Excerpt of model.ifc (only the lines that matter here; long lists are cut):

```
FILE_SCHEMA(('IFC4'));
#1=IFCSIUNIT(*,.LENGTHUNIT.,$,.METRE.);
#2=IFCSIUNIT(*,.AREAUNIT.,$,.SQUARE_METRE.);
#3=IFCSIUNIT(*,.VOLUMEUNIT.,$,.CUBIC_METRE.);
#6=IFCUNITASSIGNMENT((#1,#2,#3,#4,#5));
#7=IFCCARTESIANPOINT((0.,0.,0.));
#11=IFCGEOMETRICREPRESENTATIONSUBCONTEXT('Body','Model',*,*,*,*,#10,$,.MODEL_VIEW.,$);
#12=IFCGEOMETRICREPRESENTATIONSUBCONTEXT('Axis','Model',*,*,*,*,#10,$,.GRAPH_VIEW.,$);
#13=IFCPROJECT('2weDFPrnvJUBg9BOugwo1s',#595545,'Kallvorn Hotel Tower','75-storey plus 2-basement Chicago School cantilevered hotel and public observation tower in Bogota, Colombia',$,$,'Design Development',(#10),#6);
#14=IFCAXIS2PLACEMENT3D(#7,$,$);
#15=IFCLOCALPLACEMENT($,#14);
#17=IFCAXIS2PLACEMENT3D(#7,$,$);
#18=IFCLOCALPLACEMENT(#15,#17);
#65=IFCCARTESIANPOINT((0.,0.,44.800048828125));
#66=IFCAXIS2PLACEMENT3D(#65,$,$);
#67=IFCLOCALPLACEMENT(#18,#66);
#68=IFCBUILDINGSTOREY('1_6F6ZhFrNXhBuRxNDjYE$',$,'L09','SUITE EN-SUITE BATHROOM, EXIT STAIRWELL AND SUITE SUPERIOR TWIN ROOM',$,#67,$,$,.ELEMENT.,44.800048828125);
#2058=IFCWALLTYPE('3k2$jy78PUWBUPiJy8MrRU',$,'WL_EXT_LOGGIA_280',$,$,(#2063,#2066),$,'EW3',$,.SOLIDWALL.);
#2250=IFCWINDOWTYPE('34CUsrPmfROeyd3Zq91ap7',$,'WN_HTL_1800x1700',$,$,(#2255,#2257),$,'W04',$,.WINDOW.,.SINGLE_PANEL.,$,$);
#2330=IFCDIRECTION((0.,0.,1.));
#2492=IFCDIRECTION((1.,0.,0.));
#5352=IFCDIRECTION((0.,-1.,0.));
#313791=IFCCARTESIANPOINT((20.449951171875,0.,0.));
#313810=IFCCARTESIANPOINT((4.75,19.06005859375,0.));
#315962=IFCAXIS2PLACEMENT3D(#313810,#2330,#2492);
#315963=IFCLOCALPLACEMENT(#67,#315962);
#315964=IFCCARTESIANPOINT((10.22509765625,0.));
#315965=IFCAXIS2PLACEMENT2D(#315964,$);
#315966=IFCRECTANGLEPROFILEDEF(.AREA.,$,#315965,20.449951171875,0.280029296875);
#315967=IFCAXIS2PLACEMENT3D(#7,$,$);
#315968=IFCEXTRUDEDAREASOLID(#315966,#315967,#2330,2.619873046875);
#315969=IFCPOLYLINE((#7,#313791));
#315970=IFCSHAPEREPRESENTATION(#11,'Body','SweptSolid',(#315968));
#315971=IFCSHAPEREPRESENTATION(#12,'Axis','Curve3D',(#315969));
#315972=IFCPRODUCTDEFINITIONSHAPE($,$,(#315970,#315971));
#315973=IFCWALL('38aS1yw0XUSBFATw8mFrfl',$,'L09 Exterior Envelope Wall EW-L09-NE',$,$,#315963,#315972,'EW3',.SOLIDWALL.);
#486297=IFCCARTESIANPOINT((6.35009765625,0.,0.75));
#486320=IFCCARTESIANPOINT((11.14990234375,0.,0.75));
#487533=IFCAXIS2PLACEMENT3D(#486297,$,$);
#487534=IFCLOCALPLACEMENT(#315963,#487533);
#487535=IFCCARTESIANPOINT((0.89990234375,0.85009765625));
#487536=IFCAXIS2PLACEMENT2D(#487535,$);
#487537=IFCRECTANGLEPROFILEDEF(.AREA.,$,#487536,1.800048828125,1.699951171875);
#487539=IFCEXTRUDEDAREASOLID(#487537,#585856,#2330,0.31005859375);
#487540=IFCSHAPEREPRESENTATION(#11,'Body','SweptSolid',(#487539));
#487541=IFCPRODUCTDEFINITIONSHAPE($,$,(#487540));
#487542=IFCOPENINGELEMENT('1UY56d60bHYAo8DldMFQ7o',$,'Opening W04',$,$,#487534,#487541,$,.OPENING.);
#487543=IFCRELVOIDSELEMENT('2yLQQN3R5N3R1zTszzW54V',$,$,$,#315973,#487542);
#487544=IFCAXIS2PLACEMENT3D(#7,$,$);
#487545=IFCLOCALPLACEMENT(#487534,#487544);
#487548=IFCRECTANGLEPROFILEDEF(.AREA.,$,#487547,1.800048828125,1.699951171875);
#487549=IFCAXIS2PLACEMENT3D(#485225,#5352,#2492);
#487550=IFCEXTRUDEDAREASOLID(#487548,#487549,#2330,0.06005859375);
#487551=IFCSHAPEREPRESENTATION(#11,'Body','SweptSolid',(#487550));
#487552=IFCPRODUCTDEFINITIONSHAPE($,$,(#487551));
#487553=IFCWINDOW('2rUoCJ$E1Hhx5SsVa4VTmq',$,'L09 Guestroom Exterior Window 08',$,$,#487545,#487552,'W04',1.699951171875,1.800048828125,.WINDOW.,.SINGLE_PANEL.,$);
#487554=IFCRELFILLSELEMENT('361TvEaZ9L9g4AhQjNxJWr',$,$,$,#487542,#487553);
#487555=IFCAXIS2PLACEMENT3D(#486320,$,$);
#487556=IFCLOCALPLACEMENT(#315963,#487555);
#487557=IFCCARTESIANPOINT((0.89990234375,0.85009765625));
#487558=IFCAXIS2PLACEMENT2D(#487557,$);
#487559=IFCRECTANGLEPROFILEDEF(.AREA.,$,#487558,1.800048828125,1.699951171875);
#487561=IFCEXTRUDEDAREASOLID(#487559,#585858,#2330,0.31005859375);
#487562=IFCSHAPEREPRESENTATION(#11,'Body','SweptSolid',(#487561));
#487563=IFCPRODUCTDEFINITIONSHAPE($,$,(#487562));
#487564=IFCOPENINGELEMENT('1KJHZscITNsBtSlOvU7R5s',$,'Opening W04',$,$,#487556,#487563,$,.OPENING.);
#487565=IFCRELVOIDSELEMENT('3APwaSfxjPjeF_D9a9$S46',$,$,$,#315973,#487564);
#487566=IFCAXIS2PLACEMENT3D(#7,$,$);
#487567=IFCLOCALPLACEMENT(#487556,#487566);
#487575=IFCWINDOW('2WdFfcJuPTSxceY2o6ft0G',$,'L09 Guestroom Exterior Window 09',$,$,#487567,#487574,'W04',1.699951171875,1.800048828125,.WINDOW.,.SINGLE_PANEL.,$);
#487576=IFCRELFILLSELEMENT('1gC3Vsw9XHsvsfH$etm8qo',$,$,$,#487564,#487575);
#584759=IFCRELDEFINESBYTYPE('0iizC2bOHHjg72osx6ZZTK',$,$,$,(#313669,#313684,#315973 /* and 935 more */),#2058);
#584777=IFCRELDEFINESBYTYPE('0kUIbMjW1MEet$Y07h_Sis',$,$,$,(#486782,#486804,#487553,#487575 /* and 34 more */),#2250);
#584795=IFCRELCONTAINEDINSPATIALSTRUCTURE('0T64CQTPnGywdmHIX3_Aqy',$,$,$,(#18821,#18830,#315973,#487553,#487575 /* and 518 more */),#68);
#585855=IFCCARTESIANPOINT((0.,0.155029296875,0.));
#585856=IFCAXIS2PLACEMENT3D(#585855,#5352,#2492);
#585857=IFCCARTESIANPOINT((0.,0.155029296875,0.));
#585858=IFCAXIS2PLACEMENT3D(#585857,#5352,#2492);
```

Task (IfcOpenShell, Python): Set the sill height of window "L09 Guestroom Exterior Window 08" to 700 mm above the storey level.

```python
import numpy as np
import ifcopenshell
import ifcopenshell.api.geometry
import ifcopenshell.geom
import ifcopenshell.util.element
import ifcopenshell.util.placement
import ifcopenshell.util.shape
import ifcopenshell.util.unit

model = ifcopenshell.open("model.ifc")
unit_scale = ifcopenshell.util.unit.calculate_unit_scale(model)

window = model.by_guid("2rUoCJ$E1Hhx5SsVa4VTmq")
opening = window.FillsVoids[0].RelatingOpeningElement
storey = ifcopenshell.util.element.get_container(window, ifc_class="IfcBuildingStorey")
level = ifcopenshell.util.placement.get_local_placement(storey.ObjectPlacement)[2, 3]

# The opening's origin need not be at the sill, so measure its lowest point.
shape = ifcopenshell.geom.create_shape(ifcopenshell.geom.settings(), opening)
bottom = ifcopenshell.util.shape.get_shape_bottom_elevation(shape, shape.geometry) / unit_scale
dz = level + 0.7 / unit_scale - bottom

shift = np.array([0.0, 0.0, dz])
# The window is placed relative to its opening, so it follows when the opening moves.
matrix = ifcopenshell.util.placement.get_local_placement(opening.ObjectPlacement)
matrix[:3, 3] += shift
ifcopenshell.api.geometry.edit_object_placement(
    model, product=opening, matrix=matrix, is_si=False, should_transform_children=True
)

print(f"moved by {dz * unit_scale:+.3f} m")

model.write("model_v2.ifc")
```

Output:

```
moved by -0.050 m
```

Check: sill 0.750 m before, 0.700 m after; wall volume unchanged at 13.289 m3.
